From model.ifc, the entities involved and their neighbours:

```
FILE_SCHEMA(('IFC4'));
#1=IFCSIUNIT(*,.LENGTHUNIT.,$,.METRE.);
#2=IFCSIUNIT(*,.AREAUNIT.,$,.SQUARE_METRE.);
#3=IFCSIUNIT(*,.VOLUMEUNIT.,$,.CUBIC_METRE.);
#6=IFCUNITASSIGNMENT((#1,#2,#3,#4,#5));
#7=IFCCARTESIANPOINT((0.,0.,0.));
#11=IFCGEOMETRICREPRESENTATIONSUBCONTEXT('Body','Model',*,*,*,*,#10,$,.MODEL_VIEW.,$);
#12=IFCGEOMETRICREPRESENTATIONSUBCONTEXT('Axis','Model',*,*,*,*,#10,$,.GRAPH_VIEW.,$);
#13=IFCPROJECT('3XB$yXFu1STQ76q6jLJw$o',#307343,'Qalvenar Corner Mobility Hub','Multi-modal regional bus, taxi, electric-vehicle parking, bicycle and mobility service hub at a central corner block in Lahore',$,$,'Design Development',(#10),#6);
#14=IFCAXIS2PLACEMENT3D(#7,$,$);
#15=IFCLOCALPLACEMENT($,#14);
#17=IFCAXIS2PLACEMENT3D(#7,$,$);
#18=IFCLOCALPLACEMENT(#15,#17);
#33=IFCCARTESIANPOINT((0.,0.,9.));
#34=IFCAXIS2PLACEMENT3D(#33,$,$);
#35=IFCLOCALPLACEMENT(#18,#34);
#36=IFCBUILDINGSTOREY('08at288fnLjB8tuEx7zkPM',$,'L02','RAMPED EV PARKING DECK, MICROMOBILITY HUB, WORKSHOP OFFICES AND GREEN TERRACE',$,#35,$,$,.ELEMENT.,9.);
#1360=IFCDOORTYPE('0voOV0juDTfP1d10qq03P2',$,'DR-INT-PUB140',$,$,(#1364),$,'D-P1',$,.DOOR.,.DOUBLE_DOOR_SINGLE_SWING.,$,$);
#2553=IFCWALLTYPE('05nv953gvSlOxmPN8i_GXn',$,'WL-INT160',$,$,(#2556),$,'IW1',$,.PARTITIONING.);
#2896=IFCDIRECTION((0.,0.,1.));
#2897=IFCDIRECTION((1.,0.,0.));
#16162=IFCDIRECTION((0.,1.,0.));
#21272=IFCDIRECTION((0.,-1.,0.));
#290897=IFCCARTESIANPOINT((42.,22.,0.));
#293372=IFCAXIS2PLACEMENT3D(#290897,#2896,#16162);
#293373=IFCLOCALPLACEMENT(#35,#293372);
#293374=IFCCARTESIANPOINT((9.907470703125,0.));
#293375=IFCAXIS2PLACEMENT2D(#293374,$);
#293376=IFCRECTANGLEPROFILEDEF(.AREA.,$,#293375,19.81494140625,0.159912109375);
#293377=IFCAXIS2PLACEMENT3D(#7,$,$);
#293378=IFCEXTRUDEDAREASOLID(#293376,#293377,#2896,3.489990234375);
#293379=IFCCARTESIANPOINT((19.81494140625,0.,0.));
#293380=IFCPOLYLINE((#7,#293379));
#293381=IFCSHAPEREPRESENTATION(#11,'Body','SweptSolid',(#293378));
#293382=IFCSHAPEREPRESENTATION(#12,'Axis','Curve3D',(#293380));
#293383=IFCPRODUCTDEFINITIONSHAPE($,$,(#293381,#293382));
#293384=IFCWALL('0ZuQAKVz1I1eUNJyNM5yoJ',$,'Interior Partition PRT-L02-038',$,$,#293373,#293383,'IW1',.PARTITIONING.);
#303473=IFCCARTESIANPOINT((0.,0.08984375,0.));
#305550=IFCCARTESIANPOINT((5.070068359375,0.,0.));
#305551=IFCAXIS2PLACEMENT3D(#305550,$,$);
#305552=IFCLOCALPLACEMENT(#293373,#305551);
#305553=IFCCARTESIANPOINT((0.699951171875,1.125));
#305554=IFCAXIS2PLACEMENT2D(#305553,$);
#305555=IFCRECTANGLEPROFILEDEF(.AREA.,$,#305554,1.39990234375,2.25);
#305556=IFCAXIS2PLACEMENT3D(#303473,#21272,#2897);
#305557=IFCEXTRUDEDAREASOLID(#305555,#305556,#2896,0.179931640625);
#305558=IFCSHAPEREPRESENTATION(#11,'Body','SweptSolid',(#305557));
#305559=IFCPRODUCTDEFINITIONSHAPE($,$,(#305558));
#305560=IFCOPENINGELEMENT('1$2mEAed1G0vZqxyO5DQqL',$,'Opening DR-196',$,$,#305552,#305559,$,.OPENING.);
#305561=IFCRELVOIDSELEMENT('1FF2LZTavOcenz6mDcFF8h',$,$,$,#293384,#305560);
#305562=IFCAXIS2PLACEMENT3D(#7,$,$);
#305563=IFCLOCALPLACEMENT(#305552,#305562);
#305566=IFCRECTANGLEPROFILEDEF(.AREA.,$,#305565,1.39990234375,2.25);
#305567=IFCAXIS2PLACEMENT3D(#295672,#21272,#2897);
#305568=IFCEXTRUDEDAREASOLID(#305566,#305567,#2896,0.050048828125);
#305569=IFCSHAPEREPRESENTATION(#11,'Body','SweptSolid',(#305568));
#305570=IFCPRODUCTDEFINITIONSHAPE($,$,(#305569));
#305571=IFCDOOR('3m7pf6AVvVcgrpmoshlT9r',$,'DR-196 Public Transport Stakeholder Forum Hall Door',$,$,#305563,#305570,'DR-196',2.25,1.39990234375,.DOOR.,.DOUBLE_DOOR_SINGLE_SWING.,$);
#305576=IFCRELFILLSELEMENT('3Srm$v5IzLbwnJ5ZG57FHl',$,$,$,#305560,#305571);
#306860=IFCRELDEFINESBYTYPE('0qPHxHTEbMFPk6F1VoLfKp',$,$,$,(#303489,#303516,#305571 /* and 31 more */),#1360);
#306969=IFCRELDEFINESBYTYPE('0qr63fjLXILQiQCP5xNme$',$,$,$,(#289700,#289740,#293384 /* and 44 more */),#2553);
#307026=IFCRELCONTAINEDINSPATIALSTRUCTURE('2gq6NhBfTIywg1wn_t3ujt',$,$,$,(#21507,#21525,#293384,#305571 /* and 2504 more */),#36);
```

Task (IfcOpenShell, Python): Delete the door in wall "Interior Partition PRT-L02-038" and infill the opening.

```python
import ifcopenshell
import ifcopenshell.api.feature
import ifcopenshell.api.root
import ifcopenshell.geom
import ifcopenshell.util.shape

model = ifcopenshell.open("model.ifc")
settings = ifcopenshell.geom.settings()


def volume(element):
    """Net volume in cubic metres, openings subtracted."""
    shape = ifcopenshell.geom.create_shape(settings, element)
    return ifcopenshell.util.shape.get_volume(shape.geometry)


door = model.by_guid("3m7pf6AVvVcgrpmoshlT9r")
opening = door.FillsVoids[0].RelatingOpeningElement
wall = opening.VoidsElements[0].RelatingBuildingElement
before = volume(wall)

ifcopenshell.api.root.remove_product(model, product=door)
ifcopenshell.api.feature.remove_feature(model, feature=opening)

after = volume(wall)

print(f"wall volume {before:.3f} -> {after:.3f} m3")

model.write("model_updated.ifc")
```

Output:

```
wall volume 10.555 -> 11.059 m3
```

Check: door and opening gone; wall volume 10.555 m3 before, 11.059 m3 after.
